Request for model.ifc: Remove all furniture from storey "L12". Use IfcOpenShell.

First a look at what the model holds.

```python
import ifcopenshell
import ifcopenshell.util.element

model = ifcopenshell.open("model.ifc")
print(model.schema)
storey = next(s for s in model.by_type("IfcBuildingStorey") if s.Name == "L12")
furniture = [e for e in ifcopenshell.util.element.get_decomposition(storey) if e.is_a("IfcFurnishingElement")]
seen = {}
for e in furniture:
    element_type = ifcopenshell.util.element.get_type(e)
    name = element_type.Name if element_type not in (None, e) else None
    seen[name] = seen.get(name, 0) + 1
for name, count in sorted(seen.items(), key=str):
    print(count, "x", name)
```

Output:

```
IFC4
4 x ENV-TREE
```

```python
import ifcopenshell
import ifcopenshell.api.root
import ifcopenshell.util.element

model = ifcopenshell.open("model.ifc")

storey = next(s for s in model.by_type("IfcBuildingStorey") if s.Name == "L12")
furniture = [e for e in ifcopenshell.util.element.get_decomposition(storey) if e.is_a("IfcFurnishingElement")]

for e in furniture:
    ifcopenshell.api.root.remove_product(model, product=e)
print(len(furniture), "removed")

model.write("model_updated.ifc")
```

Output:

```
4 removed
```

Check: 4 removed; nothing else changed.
